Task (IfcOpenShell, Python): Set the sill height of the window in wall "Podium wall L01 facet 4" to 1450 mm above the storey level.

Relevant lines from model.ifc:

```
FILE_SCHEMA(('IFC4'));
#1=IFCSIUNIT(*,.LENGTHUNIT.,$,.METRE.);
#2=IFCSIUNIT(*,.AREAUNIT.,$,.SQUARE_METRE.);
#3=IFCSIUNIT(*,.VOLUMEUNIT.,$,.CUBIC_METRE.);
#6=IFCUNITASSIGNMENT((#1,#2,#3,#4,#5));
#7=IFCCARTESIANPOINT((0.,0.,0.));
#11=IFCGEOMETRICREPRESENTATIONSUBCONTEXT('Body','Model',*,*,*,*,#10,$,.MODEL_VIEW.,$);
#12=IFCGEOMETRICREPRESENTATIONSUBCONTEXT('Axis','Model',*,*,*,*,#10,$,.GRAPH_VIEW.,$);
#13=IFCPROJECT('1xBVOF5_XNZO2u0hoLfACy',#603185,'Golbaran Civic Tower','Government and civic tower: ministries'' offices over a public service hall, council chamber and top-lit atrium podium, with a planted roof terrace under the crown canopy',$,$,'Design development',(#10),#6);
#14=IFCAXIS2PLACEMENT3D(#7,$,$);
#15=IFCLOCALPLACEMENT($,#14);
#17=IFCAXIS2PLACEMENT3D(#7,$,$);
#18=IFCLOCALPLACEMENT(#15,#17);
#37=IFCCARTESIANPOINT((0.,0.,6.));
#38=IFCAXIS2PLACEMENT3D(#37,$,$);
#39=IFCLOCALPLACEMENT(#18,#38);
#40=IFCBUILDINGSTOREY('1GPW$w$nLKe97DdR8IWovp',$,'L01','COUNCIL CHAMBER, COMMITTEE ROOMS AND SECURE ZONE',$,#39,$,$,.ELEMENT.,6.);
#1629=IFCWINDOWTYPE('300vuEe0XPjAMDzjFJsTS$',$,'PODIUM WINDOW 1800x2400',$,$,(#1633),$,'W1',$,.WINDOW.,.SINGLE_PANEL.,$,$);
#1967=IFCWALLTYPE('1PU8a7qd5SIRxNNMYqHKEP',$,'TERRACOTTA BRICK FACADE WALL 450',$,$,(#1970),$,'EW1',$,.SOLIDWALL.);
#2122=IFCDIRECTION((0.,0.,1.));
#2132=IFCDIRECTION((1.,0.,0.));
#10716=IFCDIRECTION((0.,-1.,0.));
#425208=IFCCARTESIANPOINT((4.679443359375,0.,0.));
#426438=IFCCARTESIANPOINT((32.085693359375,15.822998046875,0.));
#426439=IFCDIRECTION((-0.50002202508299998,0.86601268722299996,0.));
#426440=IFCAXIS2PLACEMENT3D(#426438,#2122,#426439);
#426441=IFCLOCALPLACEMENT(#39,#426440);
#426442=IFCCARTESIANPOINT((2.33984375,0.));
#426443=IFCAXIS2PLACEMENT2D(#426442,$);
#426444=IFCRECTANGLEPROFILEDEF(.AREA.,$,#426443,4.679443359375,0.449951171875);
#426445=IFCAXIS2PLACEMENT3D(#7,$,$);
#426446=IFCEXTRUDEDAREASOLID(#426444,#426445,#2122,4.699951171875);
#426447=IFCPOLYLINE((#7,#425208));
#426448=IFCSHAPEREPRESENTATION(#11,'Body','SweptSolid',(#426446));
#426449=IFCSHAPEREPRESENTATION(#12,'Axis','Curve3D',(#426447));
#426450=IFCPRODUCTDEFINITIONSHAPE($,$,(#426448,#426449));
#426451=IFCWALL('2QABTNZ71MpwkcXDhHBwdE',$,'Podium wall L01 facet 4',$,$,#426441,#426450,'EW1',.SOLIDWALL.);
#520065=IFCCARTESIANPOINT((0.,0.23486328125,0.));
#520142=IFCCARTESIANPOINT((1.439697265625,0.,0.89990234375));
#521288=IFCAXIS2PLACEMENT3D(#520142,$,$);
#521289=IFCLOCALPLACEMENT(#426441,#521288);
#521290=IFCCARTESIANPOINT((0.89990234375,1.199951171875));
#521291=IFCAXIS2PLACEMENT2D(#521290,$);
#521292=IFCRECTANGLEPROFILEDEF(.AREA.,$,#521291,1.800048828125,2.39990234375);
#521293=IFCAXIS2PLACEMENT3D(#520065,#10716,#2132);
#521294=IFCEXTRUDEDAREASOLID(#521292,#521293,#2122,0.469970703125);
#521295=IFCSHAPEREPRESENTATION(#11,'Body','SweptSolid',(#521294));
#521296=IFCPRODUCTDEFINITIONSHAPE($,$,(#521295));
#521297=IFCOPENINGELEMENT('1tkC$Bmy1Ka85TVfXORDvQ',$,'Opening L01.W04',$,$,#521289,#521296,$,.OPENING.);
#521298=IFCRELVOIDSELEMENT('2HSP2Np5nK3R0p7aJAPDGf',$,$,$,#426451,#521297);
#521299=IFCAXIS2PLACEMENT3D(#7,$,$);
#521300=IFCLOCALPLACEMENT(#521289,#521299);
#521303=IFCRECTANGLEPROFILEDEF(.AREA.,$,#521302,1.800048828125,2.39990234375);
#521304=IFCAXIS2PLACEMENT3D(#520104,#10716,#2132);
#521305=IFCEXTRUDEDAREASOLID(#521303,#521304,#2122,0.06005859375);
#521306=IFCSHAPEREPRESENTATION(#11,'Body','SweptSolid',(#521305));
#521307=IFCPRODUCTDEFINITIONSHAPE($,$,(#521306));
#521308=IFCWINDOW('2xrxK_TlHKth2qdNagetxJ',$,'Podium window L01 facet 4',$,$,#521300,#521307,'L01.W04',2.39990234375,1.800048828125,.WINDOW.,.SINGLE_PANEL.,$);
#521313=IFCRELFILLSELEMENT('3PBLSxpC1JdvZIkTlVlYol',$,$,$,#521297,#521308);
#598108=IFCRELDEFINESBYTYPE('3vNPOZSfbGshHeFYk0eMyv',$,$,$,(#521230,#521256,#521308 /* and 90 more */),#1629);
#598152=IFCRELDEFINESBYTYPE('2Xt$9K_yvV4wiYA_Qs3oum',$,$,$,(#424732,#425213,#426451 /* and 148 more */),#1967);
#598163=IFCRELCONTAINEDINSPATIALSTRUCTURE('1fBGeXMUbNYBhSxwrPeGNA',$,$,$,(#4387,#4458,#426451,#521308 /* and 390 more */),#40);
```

```python
import numpy as np
import ifcopenshell
import ifcopenshell.api.geometry
import ifcopenshell.geom
import ifcopenshell.util.element
import ifcopenshell.util.placement
import ifcopenshell.util.shape
import ifcopenshell.util.unit

model = ifcopenshell.open("model.ifc")
unit_scale = ifcopenshell.util.unit.calculate_unit_scale(model)

window = model.by_guid("2xrxK_TlHKth2qdNagetxJ")
opening = window.FillsVoids[0].RelatingOpeningElement
storey = ifcopenshell.util.element.get_container(window, ifc_class="IfcBuildingStorey")
level = ifcopenshell.util.placement.get_local_placement(storey.ObjectPlacement)[2, 3]

# The opening's origin need not be at the sill, so measure its lowest point.
shape = ifcopenshell.geom.create_shape(ifcopenshell.geom.settings(), opening)
bottom = ifcopenshell.util.shape.get_shape_bottom_elevation(shape, shape.geometry) / unit_scale
dz = level + 1.45 / unit_scale - bottom

shift = np.array([0.0, 0.0, dz])
# The window is placed relative to its opening, so it follows when the opening moves.
matrix = ifcopenshell.util.placement.get_local_placement(opening.ObjectPlacement)
matrix[:3, 3] += shift
ifcopenshell.api.geometry.edit_object_placement(
    model, product=opening, matrix=matrix, is_si=False, should_transform_children=True
)

print(f"moved by {dz * unit_scale:+.3f} m")

model.write("model_edited.ifc")
```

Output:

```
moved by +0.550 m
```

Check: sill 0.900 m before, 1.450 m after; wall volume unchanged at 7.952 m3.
